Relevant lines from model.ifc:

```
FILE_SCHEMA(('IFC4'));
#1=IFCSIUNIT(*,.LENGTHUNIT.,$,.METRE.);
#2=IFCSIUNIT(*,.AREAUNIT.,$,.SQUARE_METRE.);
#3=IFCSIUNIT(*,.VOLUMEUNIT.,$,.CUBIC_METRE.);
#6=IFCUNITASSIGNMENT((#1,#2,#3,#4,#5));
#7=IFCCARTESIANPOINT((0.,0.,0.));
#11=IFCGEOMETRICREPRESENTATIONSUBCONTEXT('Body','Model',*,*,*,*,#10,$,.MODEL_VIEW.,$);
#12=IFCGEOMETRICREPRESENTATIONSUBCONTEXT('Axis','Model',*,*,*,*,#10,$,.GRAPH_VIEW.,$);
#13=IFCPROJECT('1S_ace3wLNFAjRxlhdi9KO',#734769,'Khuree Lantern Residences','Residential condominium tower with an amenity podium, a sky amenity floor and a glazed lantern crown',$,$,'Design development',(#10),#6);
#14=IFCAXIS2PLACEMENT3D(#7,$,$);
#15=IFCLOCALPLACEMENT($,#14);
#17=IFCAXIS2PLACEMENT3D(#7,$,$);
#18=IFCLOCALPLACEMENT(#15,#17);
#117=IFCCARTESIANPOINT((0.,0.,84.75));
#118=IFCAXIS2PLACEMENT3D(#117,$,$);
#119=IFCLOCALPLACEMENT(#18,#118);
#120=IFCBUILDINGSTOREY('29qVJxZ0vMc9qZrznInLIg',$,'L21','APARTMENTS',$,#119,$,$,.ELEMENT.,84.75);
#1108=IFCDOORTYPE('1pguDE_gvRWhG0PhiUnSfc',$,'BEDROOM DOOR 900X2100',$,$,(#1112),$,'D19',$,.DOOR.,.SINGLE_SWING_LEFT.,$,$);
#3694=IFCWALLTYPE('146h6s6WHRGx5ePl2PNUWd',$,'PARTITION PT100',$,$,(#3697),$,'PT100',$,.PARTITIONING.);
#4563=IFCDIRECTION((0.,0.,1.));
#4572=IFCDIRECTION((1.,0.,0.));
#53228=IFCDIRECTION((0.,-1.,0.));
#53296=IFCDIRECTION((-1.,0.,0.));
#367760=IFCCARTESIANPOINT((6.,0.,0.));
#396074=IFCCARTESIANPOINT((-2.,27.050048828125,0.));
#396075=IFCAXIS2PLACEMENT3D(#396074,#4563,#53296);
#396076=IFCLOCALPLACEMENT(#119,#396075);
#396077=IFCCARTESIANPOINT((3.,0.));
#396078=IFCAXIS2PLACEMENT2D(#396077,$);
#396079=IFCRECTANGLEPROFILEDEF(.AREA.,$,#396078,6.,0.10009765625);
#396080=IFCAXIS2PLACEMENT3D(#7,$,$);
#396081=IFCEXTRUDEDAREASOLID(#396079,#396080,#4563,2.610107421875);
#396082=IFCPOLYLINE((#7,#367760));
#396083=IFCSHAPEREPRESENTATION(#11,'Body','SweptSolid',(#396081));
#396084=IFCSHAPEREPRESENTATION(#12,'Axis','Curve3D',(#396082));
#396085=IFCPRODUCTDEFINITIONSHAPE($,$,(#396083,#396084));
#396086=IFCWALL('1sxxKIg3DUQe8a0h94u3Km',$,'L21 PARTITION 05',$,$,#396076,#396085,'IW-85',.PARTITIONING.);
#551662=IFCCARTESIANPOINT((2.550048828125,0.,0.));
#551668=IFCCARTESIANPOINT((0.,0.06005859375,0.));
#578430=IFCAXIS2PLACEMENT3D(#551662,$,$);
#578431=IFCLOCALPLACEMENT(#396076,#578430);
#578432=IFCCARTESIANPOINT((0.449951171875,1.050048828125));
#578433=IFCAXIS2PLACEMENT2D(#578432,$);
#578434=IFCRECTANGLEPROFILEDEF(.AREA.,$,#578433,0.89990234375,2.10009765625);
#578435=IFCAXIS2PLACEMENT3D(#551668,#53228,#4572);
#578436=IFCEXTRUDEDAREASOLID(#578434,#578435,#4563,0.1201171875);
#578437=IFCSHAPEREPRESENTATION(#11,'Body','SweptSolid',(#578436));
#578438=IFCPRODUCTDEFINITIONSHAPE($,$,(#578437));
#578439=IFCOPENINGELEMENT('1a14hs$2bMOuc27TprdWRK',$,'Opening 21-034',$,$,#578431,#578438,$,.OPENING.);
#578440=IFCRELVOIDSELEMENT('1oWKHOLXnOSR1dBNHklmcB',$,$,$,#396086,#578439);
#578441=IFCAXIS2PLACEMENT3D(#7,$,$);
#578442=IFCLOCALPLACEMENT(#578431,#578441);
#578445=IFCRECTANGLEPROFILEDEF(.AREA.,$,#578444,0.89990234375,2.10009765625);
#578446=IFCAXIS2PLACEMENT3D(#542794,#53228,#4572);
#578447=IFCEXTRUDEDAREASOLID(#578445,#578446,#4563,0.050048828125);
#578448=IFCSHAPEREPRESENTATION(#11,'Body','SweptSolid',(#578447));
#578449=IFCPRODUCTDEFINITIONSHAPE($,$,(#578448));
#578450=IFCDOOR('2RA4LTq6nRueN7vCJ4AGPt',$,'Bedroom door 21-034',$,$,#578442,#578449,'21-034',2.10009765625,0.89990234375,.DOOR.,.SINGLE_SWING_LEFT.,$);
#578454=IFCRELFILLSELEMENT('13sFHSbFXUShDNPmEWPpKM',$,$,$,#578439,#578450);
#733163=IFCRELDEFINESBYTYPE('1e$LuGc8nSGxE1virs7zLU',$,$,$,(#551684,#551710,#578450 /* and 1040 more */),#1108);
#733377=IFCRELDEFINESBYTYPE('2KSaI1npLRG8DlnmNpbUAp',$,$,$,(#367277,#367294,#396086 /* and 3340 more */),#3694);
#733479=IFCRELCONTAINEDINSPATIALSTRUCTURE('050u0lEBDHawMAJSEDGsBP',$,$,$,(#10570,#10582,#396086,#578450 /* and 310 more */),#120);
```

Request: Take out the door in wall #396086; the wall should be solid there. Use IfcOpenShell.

```python
import ifcopenshell
import ifcopenshell.api.feature
import ifcopenshell.api.root
import ifcopenshell.geom
import ifcopenshell.util.shape

model = ifcopenshell.open("model.ifc")
settings = ifcopenshell.geom.settings()


def volume(element):
    """Net volume in cubic metres, openings subtracted."""
    shape = ifcopenshell.geom.create_shape(settings, element)
    return ifcopenshell.util.shape.get_volume(shape.geometry)


door = model.by_id(578450)
opening = door.FillsVoids[0].RelatingOpeningElement
wall = opening.VoidsElements[0].RelatingBuildingElement
before = volume(wall)

ifcopenshell.api.root.remove_product(model, product=door)
ifcopenshell.api.feature.remove_feature(model, feature=opening)

after = volume(wall)

print(f"wall volume {before:.3f} -> {after:.3f} m3")

model.write("model_updated.ifc")
```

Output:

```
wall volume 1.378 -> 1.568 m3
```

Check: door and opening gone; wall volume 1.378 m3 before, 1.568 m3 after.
